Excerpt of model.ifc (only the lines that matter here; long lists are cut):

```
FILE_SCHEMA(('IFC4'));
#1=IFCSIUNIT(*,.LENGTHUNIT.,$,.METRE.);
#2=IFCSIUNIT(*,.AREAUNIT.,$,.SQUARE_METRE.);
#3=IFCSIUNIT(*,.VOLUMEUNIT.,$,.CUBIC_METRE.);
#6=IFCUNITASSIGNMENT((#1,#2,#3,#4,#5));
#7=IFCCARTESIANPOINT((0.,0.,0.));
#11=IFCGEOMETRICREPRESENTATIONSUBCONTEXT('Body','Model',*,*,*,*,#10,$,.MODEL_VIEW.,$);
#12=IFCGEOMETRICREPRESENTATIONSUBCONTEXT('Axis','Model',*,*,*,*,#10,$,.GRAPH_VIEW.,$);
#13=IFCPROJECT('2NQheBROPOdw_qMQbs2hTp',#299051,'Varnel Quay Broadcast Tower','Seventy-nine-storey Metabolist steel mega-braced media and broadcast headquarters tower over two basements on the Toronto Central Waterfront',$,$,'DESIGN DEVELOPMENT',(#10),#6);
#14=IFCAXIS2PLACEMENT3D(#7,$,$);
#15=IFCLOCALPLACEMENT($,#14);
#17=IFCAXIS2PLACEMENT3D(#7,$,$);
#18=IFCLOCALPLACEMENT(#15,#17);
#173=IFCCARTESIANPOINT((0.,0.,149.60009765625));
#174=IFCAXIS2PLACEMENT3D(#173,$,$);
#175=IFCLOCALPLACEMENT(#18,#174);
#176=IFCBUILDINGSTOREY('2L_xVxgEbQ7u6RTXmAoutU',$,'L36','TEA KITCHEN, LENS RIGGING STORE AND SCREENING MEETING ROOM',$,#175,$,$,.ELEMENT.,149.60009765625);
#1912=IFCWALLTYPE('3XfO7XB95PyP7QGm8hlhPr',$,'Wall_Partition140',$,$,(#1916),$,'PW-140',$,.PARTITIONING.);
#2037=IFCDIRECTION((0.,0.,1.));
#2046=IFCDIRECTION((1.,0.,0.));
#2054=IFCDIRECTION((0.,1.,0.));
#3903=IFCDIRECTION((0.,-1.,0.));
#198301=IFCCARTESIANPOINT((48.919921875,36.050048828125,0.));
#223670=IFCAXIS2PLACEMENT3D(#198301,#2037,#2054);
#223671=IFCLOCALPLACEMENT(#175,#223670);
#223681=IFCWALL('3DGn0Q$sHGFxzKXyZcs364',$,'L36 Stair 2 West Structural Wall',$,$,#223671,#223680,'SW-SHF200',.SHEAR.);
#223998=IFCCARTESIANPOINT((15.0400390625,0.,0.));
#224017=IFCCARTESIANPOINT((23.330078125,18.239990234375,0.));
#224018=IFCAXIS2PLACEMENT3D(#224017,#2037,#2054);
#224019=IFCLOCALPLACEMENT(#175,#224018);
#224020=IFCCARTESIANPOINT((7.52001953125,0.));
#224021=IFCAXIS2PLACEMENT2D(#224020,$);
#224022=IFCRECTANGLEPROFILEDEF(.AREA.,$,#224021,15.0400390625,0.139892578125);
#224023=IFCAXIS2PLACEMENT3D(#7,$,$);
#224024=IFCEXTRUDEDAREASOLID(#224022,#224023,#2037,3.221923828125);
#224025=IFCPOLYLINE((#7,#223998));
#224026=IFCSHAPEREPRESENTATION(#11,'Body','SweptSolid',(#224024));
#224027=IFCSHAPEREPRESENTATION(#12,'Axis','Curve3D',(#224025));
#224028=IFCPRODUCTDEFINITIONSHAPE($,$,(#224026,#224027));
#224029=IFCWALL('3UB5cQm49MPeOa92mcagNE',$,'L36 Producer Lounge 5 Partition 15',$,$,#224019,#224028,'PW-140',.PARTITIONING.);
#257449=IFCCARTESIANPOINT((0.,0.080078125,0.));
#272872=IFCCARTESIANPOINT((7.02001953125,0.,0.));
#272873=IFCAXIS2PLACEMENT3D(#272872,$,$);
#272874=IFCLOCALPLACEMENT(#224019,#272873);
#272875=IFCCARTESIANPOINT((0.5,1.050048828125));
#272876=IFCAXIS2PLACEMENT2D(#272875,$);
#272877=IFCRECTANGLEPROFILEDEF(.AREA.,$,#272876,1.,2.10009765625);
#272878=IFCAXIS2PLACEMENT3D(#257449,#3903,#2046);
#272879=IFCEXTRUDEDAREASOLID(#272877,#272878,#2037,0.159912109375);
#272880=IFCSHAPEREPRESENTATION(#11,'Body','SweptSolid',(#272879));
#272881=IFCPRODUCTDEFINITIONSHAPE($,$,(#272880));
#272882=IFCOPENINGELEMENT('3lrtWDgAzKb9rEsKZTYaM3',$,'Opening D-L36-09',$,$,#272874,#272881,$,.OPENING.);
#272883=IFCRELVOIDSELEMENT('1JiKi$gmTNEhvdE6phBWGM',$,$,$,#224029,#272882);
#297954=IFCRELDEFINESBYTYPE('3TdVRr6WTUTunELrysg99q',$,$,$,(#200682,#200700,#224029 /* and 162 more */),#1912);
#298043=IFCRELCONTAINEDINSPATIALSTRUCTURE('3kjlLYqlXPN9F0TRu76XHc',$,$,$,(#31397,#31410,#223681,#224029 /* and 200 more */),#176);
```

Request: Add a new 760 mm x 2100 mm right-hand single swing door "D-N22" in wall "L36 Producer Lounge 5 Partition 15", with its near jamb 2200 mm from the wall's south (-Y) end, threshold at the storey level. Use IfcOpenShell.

```python
import numpy as np
import ifcopenshell
import ifcopenshell.api.feature
import ifcopenshell.api.geometry
import ifcopenshell.api.root
import ifcopenshell.api.spatial
import ifcopenshell.geom
import ifcopenshell.util.element
import ifcopenshell.util.placement
import ifcopenshell.util.representation
import ifcopenshell.util.shape
import ifcopenshell.util.unit

model = ifcopenshell.open("model.ifc")
unit_scale = ifcopenshell.util.unit.calculate_unit_scale(model)
settings = ifcopenshell.geom.settings()


def volume(element):
    """Net volume in cubic metres, openings subtracted."""
    shape = ifcopenshell.geom.create_shape(settings, element)
    return ifcopenshell.util.shape.get_volume(shape.geometry)


wall = model.by_id(224029)
storey = ifcopenshell.util.element.get_container(wall, ifc_class="IfcBuildingStorey")
context = ifcopenshell.util.representation.get_context(model, "Model", "Body", "MODEL_VIEW")
before = volume(wall)

width, height, from_end, sill = 0.76, 2.1, 2.2, 0.0  # metres

# The wall runs along its own X axis, and the end named is its -X end.
wall_shape = ifcopenshell.geom.create_shape(settings, wall)
x, y, z = ifcopenshell.util.shape.get_vertices(wall_shape.geometry).T
start = x.min() + from_end
face, thickness = float(y.min()), float(y.max() - y.min())
wall_matrix = ifcopenshell.util.placement.get_local_placement(wall.ObjectPlacement)
level = ifcopenshell.util.placement.get_local_placement(storey.ObjectPlacement)[2, 3]


def in_wall(x, y):
    """Placement at x, y metres in the wall's axes, at sill height."""
    matrix = wall_matrix.copy()
    matrix[:, 3] = wall_matrix @ np.array([x / unit_scale, y / unit_scale, 0.0, 1.0])
    matrix[2, 3] = level + sill / unit_scale
    return matrix


# Opening: a box that overshoots both wall faces by 50 mm.
opening = ifcopenshell.api.root.create_entity(model, ifc_class="IfcOpeningElement", predefined_type="OPENING")
box = ifcopenshell.api.geometry.add_wall_representation(
    model, context=context, length=width, height=height, thickness=thickness + 0.1
)
ifcopenshell.api.geometry.assign_representation(model, product=opening, representation=box)
ifcopenshell.api.geometry.edit_object_placement(model, product=opening, matrix=in_wall(start, face - 0.05), is_si=False)
ifcopenshell.api.feature.add_feature(model, feature=opening, element=wall)

door = ifcopenshell.api.root.create_entity(model, ifc_class="IfcDoor", name="D-N22", predefined_type="DOOR")
door.OverallWidth, door.OverallHeight = width / unit_scale, height / unit_scale
door.OperationType = "SINGLE_SWING_RIGHT"
body = ifcopenshell.api.geometry.add_door_representation(
    model,
    context=context,
    overall_width=door.OverallWidth,
    overall_height=door.OverallHeight,
    operation_type="SINGLE_SWING_RIGHT",
    lining_properties={"LiningDepth": thickness / unit_scale, "ThresholdDepth": thickness / unit_scale},
)
ifcopenshell.api.geometry.assign_representation(model, product=door, representation=body)
ifcopenshell.api.spatial.assign_container(model, products=[door], relating_structure=storey)
ifcopenshell.api.feature.add_filling(model, opening=opening, element=door)

# The lining spans the wall, so the door starts at the wall face.
ifcopenshell.api.geometry.edit_object_placement(model, product=door, matrix=in_wall(start, face), is_si=False)

after = volume(wall)

print(f"wall volume {before:.3f} -> {after:.3f} m3")

model.write("model_v2.ifc")
```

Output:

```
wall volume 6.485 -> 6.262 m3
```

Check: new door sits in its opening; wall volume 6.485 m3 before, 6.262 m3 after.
